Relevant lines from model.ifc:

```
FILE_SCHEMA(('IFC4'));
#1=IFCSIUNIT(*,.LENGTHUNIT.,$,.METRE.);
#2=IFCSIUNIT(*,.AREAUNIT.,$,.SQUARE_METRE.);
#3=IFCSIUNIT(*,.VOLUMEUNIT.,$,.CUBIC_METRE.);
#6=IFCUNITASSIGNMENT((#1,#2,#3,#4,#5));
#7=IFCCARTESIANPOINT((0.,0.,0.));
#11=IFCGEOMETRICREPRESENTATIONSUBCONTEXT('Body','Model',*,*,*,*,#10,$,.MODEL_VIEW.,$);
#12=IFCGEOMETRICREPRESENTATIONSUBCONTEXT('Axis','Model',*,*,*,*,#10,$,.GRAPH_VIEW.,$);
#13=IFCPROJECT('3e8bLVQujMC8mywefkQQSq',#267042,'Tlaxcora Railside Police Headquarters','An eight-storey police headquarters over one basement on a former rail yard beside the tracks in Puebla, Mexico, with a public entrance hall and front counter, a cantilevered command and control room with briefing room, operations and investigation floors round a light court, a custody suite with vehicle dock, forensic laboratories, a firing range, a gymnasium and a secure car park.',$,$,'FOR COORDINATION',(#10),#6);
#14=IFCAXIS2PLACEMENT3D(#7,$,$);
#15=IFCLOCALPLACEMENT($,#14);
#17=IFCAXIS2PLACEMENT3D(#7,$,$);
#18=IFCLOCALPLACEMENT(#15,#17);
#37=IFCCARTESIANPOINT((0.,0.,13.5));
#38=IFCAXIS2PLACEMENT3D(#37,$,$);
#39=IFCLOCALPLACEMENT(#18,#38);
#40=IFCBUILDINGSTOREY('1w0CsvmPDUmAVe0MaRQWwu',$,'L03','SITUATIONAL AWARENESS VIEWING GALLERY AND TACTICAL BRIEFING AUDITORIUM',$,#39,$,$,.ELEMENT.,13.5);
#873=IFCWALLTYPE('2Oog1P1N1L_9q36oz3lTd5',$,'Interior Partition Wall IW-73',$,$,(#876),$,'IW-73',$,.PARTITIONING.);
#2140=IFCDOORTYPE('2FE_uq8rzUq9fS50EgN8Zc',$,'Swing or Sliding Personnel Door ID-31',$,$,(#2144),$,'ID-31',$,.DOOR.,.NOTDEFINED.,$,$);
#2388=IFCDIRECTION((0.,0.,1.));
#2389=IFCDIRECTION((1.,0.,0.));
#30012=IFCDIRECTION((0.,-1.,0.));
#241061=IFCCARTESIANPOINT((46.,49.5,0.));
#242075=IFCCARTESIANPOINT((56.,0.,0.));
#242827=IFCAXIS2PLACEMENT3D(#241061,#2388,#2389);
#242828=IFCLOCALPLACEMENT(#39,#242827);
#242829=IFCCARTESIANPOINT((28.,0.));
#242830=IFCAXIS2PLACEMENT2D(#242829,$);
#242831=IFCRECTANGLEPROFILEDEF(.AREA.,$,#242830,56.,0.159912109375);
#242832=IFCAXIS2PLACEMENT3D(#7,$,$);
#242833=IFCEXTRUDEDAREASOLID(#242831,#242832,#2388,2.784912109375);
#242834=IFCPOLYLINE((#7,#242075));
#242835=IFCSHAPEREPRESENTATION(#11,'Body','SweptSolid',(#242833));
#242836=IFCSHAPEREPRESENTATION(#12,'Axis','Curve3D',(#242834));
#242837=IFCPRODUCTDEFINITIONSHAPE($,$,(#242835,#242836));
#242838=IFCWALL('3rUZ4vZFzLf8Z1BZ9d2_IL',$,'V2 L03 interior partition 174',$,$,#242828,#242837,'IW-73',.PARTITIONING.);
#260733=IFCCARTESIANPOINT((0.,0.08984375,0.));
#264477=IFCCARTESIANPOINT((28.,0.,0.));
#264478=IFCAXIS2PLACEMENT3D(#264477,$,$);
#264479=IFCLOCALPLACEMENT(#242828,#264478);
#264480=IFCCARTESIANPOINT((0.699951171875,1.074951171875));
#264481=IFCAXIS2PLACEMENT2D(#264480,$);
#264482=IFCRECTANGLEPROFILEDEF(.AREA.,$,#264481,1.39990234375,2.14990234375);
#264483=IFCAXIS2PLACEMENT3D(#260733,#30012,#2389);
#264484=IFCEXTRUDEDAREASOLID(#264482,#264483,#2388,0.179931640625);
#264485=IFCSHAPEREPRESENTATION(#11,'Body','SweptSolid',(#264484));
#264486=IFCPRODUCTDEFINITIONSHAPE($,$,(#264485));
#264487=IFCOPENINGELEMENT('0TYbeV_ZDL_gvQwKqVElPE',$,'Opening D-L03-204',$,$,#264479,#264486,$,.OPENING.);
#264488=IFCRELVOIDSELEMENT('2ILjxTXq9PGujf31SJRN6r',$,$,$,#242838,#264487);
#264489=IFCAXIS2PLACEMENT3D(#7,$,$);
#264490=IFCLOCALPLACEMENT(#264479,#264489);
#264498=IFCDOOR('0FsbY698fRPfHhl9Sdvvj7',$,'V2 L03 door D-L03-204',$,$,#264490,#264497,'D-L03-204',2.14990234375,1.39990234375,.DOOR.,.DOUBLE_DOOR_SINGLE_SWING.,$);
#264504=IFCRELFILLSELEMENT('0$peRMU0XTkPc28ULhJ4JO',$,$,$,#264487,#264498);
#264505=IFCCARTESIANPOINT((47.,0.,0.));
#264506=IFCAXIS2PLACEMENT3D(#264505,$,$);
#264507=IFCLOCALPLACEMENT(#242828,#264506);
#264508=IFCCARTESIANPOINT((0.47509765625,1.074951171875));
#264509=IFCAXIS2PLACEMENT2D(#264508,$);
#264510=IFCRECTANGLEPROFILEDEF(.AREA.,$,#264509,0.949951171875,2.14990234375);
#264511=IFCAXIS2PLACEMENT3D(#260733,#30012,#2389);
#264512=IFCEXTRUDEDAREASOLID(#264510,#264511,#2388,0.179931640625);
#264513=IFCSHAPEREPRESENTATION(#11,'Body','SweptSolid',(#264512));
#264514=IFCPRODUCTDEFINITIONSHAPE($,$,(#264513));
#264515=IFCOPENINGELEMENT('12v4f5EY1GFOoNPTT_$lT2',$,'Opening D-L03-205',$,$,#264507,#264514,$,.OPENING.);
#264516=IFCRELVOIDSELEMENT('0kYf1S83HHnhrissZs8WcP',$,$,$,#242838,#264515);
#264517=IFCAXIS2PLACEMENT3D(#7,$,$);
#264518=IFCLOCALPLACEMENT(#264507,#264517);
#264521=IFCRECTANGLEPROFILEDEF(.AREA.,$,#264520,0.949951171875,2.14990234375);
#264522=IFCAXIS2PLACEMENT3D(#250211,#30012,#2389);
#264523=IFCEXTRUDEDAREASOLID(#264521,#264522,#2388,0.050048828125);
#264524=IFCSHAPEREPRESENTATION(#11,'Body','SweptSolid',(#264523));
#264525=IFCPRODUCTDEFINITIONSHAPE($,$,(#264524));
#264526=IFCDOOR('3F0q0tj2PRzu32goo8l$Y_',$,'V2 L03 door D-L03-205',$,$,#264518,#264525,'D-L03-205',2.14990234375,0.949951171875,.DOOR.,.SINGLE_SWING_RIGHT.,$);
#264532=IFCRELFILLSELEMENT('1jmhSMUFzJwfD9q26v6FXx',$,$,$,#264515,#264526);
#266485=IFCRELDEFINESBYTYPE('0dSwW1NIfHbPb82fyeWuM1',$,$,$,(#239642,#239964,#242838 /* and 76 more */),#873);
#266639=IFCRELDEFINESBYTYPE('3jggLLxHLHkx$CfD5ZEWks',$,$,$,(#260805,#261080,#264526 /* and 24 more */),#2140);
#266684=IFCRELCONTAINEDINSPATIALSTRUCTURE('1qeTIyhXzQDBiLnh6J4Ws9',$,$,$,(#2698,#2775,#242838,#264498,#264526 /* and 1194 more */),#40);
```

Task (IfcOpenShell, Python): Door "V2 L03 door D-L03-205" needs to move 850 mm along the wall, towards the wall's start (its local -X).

```python
import ifcopenshell
import ifcopenshell.api.geometry
import ifcopenshell.util.placement

model = ifcopenshell.open("model.ifc")

door = model.by_guid("3F0q0tj2PRzu32goo8l$Y_")
opening = door.FillsVoids[0].RelatingOpeningElement
wall = opening.VoidsElements[0].RelatingBuildingElement

wall_matrix = ifcopenshell.util.placement.get_local_placement(wall.ObjectPlacement)
shift = wall_matrix[:3, 0] * -0.85
before = ifcopenshell.util.placement.get_local_placement(door.ObjectPlacement)[:3, 3].copy()

# The door is placed relative to its opening, so it follows when the opening moves.
matrix = ifcopenshell.util.placement.get_local_placement(opening.ObjectPlacement)
matrix[:3, 3] += shift
ifcopenshell.api.geometry.edit_object_placement(
    model, product=opening, matrix=matrix, is_si=False, should_transform_children=True
)

after = ifcopenshell.util.placement.get_local_placement(door.ObjectPlacement)[:3, 3]
print("door moved by", (after - before).round(3) + 0.0)

model.write("model_updated.ifc")
```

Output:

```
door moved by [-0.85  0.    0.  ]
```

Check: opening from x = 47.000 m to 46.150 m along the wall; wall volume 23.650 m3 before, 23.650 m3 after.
